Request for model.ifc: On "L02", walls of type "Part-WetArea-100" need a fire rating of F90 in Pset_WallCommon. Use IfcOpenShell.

First a look at what the model holds.

```python
import ifcopenshell
import ifcopenshell.util.element

model = ifcopenshell.open("model.ifc")
print(model.schema)
storey = next(s for s in model.by_type("IfcBuildingStorey") if s.Name == "L02")
walls = [e for e in ifcopenshell.util.element.get_decomposition(storey) if e.is_a("IfcWall")]
seen = {}
for e in walls:
    element_type = ifcopenshell.util.element.get_type(e)
    key = (element_type.Name if element_type != e and element_type else None, ifcopenshell.util.element.get_pset(e, "Pset_WallCommon", "FireRating"))
    seen[key] = seen.get(key, 0) + 1
for (name, value), count in sorted(seen.items(), key=str):
    print(count, "x", name, "|", value)
```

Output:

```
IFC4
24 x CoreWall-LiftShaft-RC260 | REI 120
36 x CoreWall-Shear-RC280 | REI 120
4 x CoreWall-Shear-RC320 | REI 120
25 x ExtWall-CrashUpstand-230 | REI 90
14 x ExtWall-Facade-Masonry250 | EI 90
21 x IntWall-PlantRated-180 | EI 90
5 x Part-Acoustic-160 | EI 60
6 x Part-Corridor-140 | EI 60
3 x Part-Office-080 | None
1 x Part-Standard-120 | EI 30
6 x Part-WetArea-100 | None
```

```python
import ifcopenshell
import ifcopenshell.api.pset
import ifcopenshell.util.element

model = ifcopenshell.open("model.ifc")

storey = next(s for s in model.by_type("IfcBuildingStorey") if s.Name == "L02")
walls = [e for e in ifcopenshell.util.element.get_decomposition(storey) if e.is_a("IfcWall")]

count = 0
for e in walls:
    element_type = ifcopenshell.util.element.get_type(e)
    if element_type in (None, e) or element_type.Name != "Part-WetArea-100":
        continue
    # add_pset returns the element's existing set when there is one.
    pset = ifcopenshell.api.pset.add_pset(model, product=e, name="Pset_WallCommon")
    ifcopenshell.api.pset.edit_pset(model, pset=pset, properties={"FireRating": "F90"})
    count += 1

print(count, "walls updated")

model.write("model_updated.ifc")
```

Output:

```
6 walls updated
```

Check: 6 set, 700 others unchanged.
